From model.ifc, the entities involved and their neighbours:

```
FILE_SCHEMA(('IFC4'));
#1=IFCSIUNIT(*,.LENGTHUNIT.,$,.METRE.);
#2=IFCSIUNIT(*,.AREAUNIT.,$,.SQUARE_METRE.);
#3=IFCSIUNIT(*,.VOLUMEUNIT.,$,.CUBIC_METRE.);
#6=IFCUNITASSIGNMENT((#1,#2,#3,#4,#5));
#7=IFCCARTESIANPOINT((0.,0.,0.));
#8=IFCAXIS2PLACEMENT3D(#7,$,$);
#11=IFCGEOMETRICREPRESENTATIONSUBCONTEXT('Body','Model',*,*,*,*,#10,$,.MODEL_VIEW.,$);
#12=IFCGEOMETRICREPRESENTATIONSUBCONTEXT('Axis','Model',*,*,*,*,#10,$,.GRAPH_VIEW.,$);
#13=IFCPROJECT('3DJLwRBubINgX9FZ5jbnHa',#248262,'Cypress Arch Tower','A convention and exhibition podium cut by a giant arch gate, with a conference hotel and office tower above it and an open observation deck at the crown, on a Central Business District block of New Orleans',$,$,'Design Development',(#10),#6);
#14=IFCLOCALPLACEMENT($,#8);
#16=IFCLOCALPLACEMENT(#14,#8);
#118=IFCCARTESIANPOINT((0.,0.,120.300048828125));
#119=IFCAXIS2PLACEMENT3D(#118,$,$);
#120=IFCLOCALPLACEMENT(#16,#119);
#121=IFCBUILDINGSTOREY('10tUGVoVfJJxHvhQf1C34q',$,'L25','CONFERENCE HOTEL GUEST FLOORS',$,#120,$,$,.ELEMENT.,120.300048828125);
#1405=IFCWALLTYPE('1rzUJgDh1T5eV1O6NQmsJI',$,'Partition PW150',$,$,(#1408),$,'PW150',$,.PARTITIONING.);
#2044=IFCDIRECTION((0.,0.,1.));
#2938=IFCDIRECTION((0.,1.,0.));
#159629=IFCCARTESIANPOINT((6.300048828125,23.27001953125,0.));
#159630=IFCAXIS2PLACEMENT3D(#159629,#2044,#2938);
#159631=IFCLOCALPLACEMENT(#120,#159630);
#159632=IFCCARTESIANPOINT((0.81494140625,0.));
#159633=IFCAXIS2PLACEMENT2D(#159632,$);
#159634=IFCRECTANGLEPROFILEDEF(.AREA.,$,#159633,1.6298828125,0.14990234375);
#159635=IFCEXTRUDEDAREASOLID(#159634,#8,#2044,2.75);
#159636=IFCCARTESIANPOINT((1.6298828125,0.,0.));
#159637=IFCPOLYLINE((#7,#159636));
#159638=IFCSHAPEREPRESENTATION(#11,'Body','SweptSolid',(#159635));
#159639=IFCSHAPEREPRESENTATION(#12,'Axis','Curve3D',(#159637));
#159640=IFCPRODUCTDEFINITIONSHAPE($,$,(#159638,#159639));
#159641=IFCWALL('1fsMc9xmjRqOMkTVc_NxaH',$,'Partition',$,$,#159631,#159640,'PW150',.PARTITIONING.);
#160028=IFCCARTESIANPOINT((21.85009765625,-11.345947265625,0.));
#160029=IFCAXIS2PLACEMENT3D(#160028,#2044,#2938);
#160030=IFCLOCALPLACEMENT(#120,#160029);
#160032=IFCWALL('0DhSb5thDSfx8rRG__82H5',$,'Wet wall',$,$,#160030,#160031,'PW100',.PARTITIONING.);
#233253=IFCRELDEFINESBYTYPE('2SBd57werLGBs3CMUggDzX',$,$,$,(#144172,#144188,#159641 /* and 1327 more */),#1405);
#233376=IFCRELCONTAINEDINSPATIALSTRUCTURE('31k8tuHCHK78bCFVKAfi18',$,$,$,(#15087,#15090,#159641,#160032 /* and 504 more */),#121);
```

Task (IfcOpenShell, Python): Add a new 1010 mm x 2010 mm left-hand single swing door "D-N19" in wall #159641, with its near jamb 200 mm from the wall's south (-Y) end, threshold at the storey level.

```python
import numpy as np
import ifcopenshell
import ifcopenshell.api.feature
import ifcopenshell.api.geometry
import ifcopenshell.api.root
import ifcopenshell.api.spatial
import ifcopenshell.geom
import ifcopenshell.util.element
import ifcopenshell.util.placement
import ifcopenshell.util.representation
import ifcopenshell.util.shape
import ifcopenshell.util.unit

model = ifcopenshell.open("model.ifc")
unit_scale = ifcopenshell.util.unit.calculate_unit_scale(model)
settings = ifcopenshell.geom.settings()


def volume(element):
    """Net volume in cubic metres, openings subtracted."""
    shape = ifcopenshell.geom.create_shape(settings, element)
    return ifcopenshell.util.shape.get_volume(shape.geometry)


wall = model.by_id(159641)
storey = ifcopenshell.util.element.get_container(wall, ifc_class="IfcBuildingStorey")
context = ifcopenshell.util.representation.get_context(model, "Model", "Body", "MODEL_VIEW")
before = volume(wall)

width, height, from_end, sill = 1.01, 2.01, 0.2, 0.0  # metres

# The wall runs along its own X axis, and the end named is its -X end.
wall_shape = ifcopenshell.geom.create_shape(settings, wall)
x, y, z = ifcopenshell.util.shape.get_vertices(wall_shape.geometry).T
start = x.min() + from_end
face, thickness = float(y.min()), float(y.max() - y.min())
wall_matrix = ifcopenshell.util.placement.get_local_placement(wall.ObjectPlacement)
level = ifcopenshell.util.placement.get_local_placement(storey.ObjectPlacement)[2, 3]


def in_wall(x, y):
    """Placement at x, y metres in the wall's axes, at sill height."""
    matrix = wall_matrix.copy()
    matrix[:, 3] = wall_matrix @ np.array([x / unit_scale, y / unit_scale, 0.0, 1.0])
    matrix[2, 3] = level + sill / unit_scale
    return matrix


# Opening: a box that overshoots both wall faces by 50 mm.
opening = ifcopenshell.api.root.create_entity(model, ifc_class="IfcOpeningElement", predefined_type="OPENING")
box = ifcopenshell.api.geometry.add_wall_representation(
    model, context=context, length=width, height=height, thickness=thickness + 0.1
)
ifcopenshell.api.geometry.assign_representation(model, product=opening, representation=box)
ifcopenshell.api.geometry.edit_object_placement(model, product=opening, matrix=in_wall(start, face - 0.05), is_si=False)
ifcopenshell.api.feature.add_feature(model, feature=opening, element=wall)

door = ifcopenshell.api.root.create_entity(model, ifc_class="IfcDoor", name="D-N19", predefined_type="DOOR")
door.OverallWidth, door.OverallHeight = width / unit_scale, height / unit_scale
door.OperationType = "SINGLE_SWING_LEFT"
body = ifcopenshell.api.geometry.add_door_representation(
    model,
    context=context,
    overall_width=door.OverallWidth,
    overall_height=door.OverallHeight,
    operation_type="SINGLE_SWING_LEFT",
    lining_properties={"LiningDepth": thickness / unit_scale, "ThresholdDepth": thickness / unit_scale},
)
ifcopenshell.api.geometry.assign_representation(model, product=door, representation=body)
ifcopenshell.api.spatial.assign_container(model, products=[door], relating_structure=storey)
ifcopenshell.api.feature.add_filling(model, opening=opening, element=door)

# The lining spans the wall, so the door starts at the wall face.
ifcopenshell.api.geometry.edit_object_placement(model, product=door, matrix=in_wall(start, face), is_si=False)

after = volume(wall)

print(f"wall volume {before:.3f} -> {after:.3f} m3")

model.write("model-out.ifc")
```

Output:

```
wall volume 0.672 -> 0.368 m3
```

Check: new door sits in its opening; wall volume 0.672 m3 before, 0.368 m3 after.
